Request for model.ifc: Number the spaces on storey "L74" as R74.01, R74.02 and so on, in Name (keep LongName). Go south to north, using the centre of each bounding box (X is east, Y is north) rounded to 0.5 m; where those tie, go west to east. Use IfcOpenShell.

First a look at what the model holds.

```python
import ifcopenshell
import ifcopenshell.util.element
import ifcopenshell.util.placement

model = ifcopenshell.open("model.ifc")
print(model.schema)
storey = next(s for s in model.by_type("IfcBuildingStorey") if s.Name == "L74")
spaces = [e for e in ifcopenshell.util.element.get_decomposition(storey) if e.is_a("IfcSpace")]
for e in sorted(spaces, key=lambda e: e.id()):
    origin = ifcopenshell.util.placement.get_local_placement(e.ObjectPlacement)[:3, 3]
    print(e.id(), e.Name, e.LongName, origin.round(2) + 0.0, sep=" | ")
```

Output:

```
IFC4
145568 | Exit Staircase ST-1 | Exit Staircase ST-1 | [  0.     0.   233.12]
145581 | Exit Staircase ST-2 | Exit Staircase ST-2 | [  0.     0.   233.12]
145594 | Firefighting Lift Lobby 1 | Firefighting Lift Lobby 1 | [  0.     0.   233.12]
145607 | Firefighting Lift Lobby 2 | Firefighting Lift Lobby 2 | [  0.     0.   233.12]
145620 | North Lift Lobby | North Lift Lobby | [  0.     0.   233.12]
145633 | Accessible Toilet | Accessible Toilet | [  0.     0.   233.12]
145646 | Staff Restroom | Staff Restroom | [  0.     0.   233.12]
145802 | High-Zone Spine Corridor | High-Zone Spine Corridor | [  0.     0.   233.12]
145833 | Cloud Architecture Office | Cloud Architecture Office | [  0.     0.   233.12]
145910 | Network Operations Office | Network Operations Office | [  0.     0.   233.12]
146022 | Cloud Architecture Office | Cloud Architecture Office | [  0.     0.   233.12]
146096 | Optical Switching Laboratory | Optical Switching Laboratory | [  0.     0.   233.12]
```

```python
import ifcopenshell
import ifcopenshell.geom
import ifcopenshell.util.element
import ifcopenshell.util.shape

model = ifcopenshell.open("model.ifc")
settings = ifcopenshell.geom.settings()
settings.set("use-world-coords", True)


def centre(element):
    shape = ifcopenshell.geom.create_shape(settings, element)
    return ifcopenshell.util.shape.get_bbox_centroid(shape.geometry)


storey = next(s for s in model.by_type("IfcBuildingStorey") if s.Name == "L74")
spaces = [e for e in ifcopenshell.util.element.get_decomposition(storey) if e.is_a("IfcSpace")]

# Insertion points can sit at a corner or the storey origin, so sort by the geometry (in metres).
centres = {e: centre(e) for e in spaces}
spaces.sort(key=lambda e: (round(centres[e][1] / 0.5), centres[e][0]))

for i, e in enumerate(spaces, start=1):
    number = f"R74.{i:02d}"
    e.Name = number
    print(e.id(), number)

model.write("model_updated.ifc")
```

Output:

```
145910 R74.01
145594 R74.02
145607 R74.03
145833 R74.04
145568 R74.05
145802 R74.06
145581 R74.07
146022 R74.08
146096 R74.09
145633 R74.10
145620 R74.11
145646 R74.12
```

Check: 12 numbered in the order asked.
